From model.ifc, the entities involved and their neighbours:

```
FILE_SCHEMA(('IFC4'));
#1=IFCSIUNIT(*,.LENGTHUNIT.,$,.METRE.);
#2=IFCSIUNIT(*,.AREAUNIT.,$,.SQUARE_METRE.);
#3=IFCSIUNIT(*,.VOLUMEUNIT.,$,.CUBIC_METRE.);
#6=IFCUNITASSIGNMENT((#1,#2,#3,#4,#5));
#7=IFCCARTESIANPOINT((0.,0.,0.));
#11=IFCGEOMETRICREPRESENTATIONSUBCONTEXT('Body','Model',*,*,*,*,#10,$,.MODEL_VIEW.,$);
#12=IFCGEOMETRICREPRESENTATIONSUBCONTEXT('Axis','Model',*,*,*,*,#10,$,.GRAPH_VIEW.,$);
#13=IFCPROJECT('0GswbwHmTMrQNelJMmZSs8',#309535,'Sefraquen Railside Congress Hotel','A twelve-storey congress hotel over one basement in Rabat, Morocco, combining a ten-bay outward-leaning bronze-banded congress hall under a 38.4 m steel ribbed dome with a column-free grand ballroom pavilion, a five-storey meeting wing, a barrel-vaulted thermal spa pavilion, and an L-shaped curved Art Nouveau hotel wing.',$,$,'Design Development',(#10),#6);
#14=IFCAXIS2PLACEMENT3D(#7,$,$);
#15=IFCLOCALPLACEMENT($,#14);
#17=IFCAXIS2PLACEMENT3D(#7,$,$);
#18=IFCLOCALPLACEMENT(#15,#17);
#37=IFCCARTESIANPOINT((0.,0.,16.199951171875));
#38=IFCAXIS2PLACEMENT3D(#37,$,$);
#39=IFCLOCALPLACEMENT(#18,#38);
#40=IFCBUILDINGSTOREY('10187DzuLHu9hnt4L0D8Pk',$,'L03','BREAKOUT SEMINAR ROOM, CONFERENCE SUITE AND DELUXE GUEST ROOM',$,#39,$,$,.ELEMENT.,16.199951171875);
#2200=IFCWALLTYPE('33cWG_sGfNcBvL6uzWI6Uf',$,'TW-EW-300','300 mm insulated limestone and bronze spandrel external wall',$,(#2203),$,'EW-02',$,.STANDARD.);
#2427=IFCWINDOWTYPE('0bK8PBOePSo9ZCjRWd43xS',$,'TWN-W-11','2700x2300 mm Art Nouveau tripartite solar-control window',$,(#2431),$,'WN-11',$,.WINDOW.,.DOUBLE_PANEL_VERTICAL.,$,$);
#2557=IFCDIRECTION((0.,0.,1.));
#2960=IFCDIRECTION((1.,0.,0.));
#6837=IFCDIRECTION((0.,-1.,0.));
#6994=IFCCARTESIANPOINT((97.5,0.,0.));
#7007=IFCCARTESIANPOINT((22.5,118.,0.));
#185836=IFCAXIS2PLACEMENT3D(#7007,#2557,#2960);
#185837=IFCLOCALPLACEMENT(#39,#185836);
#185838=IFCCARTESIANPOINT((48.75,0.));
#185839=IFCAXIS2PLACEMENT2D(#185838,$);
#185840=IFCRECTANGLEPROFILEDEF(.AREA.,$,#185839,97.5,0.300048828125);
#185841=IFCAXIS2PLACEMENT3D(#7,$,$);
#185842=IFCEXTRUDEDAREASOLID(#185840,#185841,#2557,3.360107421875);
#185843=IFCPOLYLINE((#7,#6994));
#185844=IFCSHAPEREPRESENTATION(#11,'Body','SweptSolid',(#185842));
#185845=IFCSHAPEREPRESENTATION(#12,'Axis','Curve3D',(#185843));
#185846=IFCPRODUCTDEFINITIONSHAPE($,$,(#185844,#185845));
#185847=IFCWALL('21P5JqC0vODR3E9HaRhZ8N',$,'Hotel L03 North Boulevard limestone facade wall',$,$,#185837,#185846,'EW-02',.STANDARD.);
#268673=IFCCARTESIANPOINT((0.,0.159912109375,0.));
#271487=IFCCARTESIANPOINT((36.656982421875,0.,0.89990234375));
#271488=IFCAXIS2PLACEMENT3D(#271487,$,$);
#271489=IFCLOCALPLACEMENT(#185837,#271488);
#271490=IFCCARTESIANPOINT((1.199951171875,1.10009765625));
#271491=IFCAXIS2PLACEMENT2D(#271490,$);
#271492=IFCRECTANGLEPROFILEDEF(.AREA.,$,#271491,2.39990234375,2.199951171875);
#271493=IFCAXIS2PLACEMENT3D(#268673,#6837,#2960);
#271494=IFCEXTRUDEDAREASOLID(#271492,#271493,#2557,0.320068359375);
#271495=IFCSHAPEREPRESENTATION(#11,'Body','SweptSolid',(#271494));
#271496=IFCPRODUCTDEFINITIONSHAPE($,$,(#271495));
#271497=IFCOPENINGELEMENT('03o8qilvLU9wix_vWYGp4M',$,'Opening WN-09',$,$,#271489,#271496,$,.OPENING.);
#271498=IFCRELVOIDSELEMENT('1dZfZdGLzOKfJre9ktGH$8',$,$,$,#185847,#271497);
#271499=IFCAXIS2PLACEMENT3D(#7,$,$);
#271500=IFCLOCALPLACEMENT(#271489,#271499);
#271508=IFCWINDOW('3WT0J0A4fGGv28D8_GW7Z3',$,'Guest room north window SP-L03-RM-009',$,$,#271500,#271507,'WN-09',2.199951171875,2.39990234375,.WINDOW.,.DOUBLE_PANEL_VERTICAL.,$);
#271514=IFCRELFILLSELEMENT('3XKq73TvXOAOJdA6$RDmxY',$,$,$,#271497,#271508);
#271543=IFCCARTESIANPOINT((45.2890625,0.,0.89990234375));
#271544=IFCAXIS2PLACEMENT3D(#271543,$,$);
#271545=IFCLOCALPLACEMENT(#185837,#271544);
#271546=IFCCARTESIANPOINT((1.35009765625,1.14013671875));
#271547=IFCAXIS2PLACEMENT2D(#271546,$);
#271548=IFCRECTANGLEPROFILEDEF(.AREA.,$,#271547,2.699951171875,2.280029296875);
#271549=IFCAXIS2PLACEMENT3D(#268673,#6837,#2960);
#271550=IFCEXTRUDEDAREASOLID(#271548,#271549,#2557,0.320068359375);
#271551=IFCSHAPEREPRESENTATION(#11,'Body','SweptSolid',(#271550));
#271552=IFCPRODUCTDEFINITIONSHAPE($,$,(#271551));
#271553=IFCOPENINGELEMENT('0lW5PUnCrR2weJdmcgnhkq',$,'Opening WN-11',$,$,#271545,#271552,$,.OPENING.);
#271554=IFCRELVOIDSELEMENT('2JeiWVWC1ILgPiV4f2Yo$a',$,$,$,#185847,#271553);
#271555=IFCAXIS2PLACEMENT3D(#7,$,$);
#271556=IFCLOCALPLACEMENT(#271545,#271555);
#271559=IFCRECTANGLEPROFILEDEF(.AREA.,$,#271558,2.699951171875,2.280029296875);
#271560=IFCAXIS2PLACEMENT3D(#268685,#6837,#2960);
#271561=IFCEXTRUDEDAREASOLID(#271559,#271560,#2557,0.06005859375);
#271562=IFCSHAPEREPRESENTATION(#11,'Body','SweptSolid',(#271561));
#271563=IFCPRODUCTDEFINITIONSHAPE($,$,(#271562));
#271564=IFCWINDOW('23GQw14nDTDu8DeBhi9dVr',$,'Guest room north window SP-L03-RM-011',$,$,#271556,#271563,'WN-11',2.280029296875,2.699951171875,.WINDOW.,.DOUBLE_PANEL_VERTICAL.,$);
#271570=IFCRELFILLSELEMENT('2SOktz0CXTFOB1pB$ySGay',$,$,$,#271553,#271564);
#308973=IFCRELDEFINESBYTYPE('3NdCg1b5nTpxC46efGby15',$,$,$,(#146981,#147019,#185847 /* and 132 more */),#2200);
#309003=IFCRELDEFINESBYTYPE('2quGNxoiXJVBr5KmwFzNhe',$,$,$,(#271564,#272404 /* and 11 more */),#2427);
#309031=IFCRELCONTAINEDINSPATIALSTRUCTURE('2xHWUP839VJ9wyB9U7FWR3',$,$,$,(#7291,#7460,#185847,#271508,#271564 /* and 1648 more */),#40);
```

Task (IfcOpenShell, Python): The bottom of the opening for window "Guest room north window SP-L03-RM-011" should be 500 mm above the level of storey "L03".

```python
import numpy as np
import ifcopenshell
import ifcopenshell.api.geometry
import ifcopenshell.geom
import ifcopenshell.util.element
import ifcopenshell.util.placement
import ifcopenshell.util.shape
import ifcopenshell.util.unit

model = ifcopenshell.open("model.ifc")
unit_scale = ifcopenshell.util.unit.calculate_unit_scale(model)

window = model.by_guid("23GQw14nDTDu8DeBhi9dVr")
opening = window.FillsVoids[0].RelatingOpeningElement
storey = ifcopenshell.util.element.get_container(window, ifc_class="IfcBuildingStorey")
level = ifcopenshell.util.placement.get_local_placement(storey.ObjectPlacement)[2, 3]

# The opening's origin need not be at the sill, so measure its lowest point.
shape = ifcopenshell.geom.create_shape(ifcopenshell.geom.settings(), opening)
bottom = ifcopenshell.util.shape.get_shape_bottom_elevation(shape, shape.geometry) / unit_scale
dz = level + 0.5 / unit_scale - bottom

shift = np.array([0.0, 0.0, dz])
# The window is placed relative to its opening, so it follows when the opening moves.
matrix = ifcopenshell.util.placement.get_local_placement(opening.ObjectPlacement)
matrix[:3, 3] += shift
ifcopenshell.api.geometry.edit_object_placement(
    model, product=opening, matrix=matrix, is_si=False, should_transform_children=True
)

print(f"moved by {dz * unit_scale:+.3f} m")

model.write("model_rev.ifc")
```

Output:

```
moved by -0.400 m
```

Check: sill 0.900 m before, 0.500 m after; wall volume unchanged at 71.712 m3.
